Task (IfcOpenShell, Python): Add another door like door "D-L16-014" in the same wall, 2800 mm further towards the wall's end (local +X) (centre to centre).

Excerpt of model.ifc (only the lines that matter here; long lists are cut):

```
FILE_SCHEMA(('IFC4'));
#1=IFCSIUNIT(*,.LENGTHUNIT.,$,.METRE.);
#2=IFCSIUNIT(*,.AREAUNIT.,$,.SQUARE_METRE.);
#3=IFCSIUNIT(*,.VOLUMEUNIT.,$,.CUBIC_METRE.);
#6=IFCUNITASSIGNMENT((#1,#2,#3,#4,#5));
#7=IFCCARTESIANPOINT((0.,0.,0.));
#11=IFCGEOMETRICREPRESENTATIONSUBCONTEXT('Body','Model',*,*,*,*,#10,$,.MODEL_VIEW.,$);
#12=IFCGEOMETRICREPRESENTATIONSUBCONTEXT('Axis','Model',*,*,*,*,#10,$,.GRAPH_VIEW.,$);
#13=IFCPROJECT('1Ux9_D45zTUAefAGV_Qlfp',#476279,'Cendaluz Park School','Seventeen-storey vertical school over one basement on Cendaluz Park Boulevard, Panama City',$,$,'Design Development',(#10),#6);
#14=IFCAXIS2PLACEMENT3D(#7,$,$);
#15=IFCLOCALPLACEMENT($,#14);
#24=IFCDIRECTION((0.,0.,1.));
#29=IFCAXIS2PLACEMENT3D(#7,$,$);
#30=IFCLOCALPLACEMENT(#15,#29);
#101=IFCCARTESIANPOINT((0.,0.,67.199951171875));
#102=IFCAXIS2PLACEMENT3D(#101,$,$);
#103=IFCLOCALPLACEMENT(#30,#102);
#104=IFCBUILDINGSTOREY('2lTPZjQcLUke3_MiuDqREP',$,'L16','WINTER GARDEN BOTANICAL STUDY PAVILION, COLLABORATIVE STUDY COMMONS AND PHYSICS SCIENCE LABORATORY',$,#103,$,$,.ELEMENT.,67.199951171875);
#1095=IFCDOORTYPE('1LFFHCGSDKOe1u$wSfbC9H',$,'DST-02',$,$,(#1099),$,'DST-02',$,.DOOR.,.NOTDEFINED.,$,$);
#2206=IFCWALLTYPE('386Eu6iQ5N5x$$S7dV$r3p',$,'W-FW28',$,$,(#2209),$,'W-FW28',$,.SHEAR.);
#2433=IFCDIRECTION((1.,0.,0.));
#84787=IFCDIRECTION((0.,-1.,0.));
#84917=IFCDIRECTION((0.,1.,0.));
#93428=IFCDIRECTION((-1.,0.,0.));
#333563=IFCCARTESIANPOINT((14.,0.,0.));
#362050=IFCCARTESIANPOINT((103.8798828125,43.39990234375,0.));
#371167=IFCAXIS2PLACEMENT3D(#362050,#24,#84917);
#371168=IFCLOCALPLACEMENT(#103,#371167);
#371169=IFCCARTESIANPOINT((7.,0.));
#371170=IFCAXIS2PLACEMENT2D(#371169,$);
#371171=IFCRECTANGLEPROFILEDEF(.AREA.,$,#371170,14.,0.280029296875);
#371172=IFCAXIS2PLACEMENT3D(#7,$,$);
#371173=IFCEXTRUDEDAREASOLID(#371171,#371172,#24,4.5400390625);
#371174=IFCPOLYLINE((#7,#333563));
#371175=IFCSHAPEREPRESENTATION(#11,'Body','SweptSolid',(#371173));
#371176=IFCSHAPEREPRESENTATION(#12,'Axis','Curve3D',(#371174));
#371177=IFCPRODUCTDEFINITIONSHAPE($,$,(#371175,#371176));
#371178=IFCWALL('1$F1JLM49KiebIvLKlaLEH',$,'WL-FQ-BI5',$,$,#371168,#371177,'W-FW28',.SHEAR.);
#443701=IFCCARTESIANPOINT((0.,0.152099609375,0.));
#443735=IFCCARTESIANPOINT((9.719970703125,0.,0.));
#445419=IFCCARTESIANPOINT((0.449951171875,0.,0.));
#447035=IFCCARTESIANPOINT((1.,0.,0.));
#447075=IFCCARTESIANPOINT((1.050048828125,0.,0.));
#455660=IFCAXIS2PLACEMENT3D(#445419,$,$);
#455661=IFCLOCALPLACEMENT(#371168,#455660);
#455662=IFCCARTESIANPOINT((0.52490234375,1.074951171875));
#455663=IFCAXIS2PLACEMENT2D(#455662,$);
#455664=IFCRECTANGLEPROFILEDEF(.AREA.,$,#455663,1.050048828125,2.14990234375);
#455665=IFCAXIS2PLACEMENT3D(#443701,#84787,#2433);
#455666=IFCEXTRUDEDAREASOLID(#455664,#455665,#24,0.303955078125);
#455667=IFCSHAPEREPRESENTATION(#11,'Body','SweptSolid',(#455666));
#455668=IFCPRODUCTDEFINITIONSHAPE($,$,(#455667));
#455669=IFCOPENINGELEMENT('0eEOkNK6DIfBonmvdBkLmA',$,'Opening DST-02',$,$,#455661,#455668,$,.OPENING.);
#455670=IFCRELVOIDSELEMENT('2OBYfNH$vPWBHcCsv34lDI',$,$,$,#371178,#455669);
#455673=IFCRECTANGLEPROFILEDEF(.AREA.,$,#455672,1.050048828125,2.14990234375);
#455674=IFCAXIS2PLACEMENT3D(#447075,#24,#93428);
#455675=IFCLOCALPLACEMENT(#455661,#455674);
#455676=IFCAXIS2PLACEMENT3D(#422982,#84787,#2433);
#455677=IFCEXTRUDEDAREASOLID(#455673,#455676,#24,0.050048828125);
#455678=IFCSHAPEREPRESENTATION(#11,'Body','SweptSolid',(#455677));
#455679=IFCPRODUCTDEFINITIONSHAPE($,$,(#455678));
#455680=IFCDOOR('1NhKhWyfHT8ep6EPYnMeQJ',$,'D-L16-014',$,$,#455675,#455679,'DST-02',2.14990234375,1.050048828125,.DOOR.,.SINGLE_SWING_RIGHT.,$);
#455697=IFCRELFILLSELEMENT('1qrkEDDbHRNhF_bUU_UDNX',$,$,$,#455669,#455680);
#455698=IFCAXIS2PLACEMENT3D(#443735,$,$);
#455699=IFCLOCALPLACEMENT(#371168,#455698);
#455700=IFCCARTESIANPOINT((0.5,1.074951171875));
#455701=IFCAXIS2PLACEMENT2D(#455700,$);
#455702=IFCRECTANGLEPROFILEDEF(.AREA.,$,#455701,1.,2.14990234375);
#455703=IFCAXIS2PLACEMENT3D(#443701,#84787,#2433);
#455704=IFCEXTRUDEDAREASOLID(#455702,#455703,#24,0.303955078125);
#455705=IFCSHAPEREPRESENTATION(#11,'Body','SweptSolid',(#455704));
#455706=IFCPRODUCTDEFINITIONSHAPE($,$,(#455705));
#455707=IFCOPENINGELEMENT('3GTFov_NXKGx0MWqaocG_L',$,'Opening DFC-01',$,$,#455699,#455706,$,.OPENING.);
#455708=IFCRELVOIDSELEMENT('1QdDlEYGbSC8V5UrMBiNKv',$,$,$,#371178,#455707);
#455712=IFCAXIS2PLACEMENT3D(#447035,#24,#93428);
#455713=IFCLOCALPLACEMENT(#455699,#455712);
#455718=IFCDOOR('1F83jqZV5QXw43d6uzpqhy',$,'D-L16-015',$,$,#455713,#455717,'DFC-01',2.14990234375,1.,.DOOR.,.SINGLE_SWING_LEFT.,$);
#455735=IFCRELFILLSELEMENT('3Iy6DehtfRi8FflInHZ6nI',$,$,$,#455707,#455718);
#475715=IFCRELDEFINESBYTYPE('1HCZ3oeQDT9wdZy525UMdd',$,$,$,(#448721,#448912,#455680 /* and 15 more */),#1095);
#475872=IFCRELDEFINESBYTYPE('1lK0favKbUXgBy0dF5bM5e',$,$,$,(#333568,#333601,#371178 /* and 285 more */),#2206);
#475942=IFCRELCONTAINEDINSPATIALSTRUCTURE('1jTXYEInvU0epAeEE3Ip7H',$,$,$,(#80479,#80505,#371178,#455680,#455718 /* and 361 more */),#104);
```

```python
import ifcopenshell
import ifcopenshell.api.feature
import ifcopenshell.api.geometry
import ifcopenshell.api.root
import ifcopenshell.geom
import ifcopenshell.util.element
import ifcopenshell.util.placement
import ifcopenshell.util.shape
import ifcopenshell.util.unit

model = ifcopenshell.open("model.ifc")
unit_scale = ifcopenshell.util.unit.calculate_unit_scale(model)
settings = ifcopenshell.geom.settings()


def volume(element):
    """Net volume in cubic metres, openings subtracted."""
    shape = ifcopenshell.geom.create_shape(settings, element)
    return ifcopenshell.util.shape.get_volume(shape.geometry)


door = model.by_guid("1NhKhWyfHT8ep6EPYnMeQJ")
opening = door.FillsVoids[0].RelatingOpeningElement
wall = opening.VoidsElements[0].RelatingBuildingElement
before = volume(wall)
shift = ifcopenshell.util.placement.get_local_placement(wall.ObjectPlacement)[:3, 0] * 2.8 / unit_scale

# copy_class copies the void relationship, type, container and properties, but no geometry.
new_opening = ifcopenshell.api.root.copy_class(model, product=opening)
new_opening.Representation = ifcopenshell.util.element.copy_deep(
    model, opening.Representation, exclude=["IfcGeometricRepresentationContext", "IfcRepresentationMap"]
)
new_door = ifcopenshell.api.root.copy_class(model, product=door)
new_door.Representation = ifcopenshell.util.element.copy_deep(
    model, door.Representation, exclude=["IfcGeometricRepresentationContext", "IfcRepresentationMap"]
)
new_door.Tag = None
ifcopenshell.api.feature.add_filling(model, opening=new_opening, element=new_door)

for old, new in ((opening, new_opening), (door, new_door)):
    matrix = ifcopenshell.util.placement.get_local_placement(old.ObjectPlacement)
    matrix[:3, 3] += shift
    ifcopenshell.api.geometry.edit_object_placement(model, product=new, matrix=matrix, is_si=False)

after = volume(wall)

print(f"wall volume {before:.3f} -> {after:.3f} m3")

model.write("model_edited.ifc")
```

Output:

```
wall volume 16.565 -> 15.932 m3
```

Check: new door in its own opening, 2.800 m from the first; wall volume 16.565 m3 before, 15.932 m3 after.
